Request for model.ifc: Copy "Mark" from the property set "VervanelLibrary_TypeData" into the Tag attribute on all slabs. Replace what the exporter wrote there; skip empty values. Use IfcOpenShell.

First a look at what the model holds.

```python
import ifcopenshell
import ifcopenshell.util.element

model = ifcopenshell.open("model.ifc")
print(model.schema)
slabs = model.by_type("IfcSlab")
print(len(slabs), "slabs")
for e in slabs[:8]:
    source = ifcopenshell.util.element.get_pset(e, "VervanelLibrary_TypeData", "Mark")
    target = e.Tag
    print(e.id(), repr(source), repr(target), sep=" | ")
```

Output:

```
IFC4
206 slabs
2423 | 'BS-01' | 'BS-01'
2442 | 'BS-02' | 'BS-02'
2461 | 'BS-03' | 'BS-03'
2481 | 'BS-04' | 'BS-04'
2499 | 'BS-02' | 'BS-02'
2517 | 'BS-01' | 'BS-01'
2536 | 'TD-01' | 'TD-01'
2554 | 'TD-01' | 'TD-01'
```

```python
import ifcopenshell
import ifcopenshell.util.element

model = ifcopenshell.open("model.ifc")

count = 0
for e in model.by_type("IfcSlab"):
    value = ifcopenshell.util.element.get_pset(e, "VervanelLibrary_TypeData", "Mark")
    current = e.Tag
    if not value or not value.strip() or current == value:
        continue
    e.Tag = value
    count += 1

print(count, "slabs updated")

model.write("model_rev.ifc")
```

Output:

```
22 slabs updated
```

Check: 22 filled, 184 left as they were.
